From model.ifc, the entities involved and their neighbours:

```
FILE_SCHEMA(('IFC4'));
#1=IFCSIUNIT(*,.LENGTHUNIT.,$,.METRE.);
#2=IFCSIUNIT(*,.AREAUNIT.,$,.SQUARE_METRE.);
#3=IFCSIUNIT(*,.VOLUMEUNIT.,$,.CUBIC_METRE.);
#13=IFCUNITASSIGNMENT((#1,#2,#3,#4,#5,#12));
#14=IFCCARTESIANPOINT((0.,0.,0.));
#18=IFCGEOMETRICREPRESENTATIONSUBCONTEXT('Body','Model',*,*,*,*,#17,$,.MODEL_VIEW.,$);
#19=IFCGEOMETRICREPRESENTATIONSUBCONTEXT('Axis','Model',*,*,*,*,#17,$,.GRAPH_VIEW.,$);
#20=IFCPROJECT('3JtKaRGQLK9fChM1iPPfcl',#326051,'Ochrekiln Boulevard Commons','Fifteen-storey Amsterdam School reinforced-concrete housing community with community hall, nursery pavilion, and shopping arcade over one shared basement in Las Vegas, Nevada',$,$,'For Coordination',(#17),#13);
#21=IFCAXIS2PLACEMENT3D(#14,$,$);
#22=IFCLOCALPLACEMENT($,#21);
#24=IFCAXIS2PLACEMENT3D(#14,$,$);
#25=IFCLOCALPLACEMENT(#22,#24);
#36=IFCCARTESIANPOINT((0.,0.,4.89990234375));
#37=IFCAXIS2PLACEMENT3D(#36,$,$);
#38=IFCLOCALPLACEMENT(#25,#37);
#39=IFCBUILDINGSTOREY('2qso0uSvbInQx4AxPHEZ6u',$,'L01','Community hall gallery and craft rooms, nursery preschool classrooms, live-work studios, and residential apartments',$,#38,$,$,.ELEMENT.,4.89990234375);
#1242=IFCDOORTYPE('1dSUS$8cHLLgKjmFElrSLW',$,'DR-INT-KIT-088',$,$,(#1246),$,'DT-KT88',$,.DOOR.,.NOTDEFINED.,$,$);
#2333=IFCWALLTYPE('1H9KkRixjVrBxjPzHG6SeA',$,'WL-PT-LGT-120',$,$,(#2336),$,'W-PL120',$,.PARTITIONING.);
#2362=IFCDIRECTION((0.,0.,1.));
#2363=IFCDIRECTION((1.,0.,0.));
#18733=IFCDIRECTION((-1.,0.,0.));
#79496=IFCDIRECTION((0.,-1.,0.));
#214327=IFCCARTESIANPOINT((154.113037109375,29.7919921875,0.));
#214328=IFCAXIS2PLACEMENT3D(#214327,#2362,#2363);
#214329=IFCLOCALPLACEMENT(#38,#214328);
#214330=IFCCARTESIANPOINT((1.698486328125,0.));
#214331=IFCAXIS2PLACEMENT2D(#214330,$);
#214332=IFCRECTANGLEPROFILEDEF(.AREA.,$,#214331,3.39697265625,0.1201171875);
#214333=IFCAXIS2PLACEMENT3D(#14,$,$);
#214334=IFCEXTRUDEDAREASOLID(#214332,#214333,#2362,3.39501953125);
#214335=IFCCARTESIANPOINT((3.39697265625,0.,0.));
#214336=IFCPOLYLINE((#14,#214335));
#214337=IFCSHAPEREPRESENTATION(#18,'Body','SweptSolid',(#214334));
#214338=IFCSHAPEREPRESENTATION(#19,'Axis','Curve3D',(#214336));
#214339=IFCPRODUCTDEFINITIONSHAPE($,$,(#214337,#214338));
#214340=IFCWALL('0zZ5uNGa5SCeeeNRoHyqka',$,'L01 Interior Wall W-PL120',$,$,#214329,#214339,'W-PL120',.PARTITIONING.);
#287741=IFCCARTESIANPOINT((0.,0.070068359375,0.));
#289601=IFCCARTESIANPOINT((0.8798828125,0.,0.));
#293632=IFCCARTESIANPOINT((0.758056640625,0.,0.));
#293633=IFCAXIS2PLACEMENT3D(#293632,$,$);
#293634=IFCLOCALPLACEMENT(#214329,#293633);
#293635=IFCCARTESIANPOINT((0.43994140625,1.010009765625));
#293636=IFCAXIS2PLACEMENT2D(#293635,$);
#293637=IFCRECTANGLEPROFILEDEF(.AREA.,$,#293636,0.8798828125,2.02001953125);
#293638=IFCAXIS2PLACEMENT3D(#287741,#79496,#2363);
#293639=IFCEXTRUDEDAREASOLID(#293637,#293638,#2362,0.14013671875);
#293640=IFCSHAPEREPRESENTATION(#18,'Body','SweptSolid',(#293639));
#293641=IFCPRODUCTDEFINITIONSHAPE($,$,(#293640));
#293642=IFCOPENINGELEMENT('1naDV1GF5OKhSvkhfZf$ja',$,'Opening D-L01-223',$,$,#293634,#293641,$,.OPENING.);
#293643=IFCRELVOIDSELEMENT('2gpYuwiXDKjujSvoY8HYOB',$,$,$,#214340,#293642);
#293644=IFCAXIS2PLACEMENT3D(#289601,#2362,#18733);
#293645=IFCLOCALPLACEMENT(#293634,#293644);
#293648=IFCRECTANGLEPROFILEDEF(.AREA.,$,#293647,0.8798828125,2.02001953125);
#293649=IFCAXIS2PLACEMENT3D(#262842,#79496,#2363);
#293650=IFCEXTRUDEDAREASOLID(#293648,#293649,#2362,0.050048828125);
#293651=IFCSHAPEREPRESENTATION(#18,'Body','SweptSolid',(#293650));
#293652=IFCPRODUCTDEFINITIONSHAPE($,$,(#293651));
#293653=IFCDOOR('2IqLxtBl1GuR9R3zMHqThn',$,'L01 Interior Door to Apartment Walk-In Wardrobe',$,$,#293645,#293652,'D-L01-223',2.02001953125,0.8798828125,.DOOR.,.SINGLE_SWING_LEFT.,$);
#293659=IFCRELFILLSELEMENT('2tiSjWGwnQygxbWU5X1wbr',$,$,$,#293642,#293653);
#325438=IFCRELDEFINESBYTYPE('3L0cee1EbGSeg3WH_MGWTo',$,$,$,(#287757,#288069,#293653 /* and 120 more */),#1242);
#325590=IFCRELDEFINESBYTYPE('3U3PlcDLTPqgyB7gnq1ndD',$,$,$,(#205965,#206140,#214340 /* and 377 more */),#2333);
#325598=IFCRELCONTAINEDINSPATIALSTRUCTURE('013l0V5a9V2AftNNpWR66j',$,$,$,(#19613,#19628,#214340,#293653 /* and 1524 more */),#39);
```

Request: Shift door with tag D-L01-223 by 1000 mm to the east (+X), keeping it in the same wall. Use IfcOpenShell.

```python
import ifcopenshell
import ifcopenshell.api.geometry
import ifcopenshell.util.placement

model = ifcopenshell.open("model.ifc")

door = model.by_id(293653)
opening = door.FillsVoids[0].RelatingOpeningElement
wall = opening.VoidsElements[0].RelatingBuildingElement

wall_matrix = ifcopenshell.util.placement.get_local_placement(wall.ObjectPlacement)
shift = wall_matrix[:3, 0] * 1.0
before = ifcopenshell.util.placement.get_local_placement(door.ObjectPlacement)[:3, 3].copy()

# The door is placed relative to its opening, so it follows when the opening moves.
matrix = ifcopenshell.util.placement.get_local_placement(opening.ObjectPlacement)
matrix[:3, 3] += shift
ifcopenshell.api.geometry.edit_object_placement(
    model, product=opening, matrix=matrix, is_si=False, should_transform_children=True
)

after = ifcopenshell.util.placement.get_local_placement(door.ObjectPlacement)[:3, 3]
print("door moved by", (after - before).round(3) + 0.0)

model.write("model_updated.ifc")
```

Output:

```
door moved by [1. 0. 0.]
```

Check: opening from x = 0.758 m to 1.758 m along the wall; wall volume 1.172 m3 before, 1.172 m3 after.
